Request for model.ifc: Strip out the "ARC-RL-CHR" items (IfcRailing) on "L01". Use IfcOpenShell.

First a look at what the model holds.

```python
import ifcopenshell
import ifcopenshell.util.element

model = ifcopenshell.open("model.ifc")
print(model.schema)
storey = next(s for s in model.by_type("IfcBuildingStorey") if s.Name == "L01")
railings = [e for e in ifcopenshell.util.element.get_decomposition(storey) if e.is_a("IfcRailing")]
seen = {}
for e in railings:
    element_type = ifcopenshell.util.element.get_type(e)
    name = element_type.Name if element_type not in (None, e) else None
    seen[name] = seen.get(name, 0) + 1
for name, count in sorted(seen.items(), key=str):
    print(count, "x", name)
```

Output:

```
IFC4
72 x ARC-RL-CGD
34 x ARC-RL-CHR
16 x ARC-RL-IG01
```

```python
import ifcopenshell
import ifcopenshell.api.root
import ifcopenshell.util.element

model = ifcopenshell.open("model.ifc")

storey = next(s for s in model.by_type("IfcBuildingStorey") if s.Name == "L01")
railings = [e for e in ifcopenshell.util.element.get_decomposition(storey) if e.is_a("IfcRailing")]
targets = [e for e in railings if (t := ifcopenshell.util.element.get_type(e)) not in (None, e) and t.Name == "ARC-RL-CHR"]

for e in targets:
    ifcopenshell.api.root.remove_product(model, product=e)
print(len(targets), "removed")

model.write("model_updated.ifc")
```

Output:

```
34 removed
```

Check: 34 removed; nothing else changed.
